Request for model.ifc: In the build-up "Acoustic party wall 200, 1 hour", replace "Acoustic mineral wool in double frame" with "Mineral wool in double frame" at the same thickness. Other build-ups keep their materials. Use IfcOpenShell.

First a look at what the model holds.

```python
import ifcopenshell
import ifcopenshell.util.element

model = ifcopenshell.open("model.ifc")
print(model.schema)
for layer_set in model.by_type("IfcMaterialLayerSet"):
    if layer_set.LayerSetName == "Acoustic party wall 200, 1 hour":
        for layer in layer_set.MaterialLayers:
            print(layer.id(), layer.Material and layer.Material.Name, layer.LayerThickness, sep=" | ")
        print(len(ifcopenshell.util.element.get_elements_by_material(model, layer_set)), "elements and types use it")
print(sorted(m.Name for m in model.by_type("IfcMaterial") if m.Name)[:60])
```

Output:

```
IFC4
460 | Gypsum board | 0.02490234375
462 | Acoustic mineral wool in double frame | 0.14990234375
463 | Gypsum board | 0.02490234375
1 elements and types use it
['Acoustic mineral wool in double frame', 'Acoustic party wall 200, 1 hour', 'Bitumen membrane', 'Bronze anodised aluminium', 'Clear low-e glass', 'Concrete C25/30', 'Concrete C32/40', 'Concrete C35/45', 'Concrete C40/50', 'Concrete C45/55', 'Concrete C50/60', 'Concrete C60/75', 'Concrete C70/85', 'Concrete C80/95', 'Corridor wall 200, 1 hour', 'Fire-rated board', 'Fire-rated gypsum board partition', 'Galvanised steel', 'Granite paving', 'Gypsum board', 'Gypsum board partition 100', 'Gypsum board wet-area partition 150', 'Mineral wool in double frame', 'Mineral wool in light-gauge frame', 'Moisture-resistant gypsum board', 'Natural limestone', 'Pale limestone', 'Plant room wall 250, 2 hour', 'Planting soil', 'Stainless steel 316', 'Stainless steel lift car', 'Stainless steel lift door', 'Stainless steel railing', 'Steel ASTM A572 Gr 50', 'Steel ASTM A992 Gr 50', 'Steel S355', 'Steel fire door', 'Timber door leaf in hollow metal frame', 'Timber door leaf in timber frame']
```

```python
import ifcopenshell
import ifcopenshell.api.material

model = ifcopenshell.open("model.ifc")

layer_set = next(s for s in model.by_type("IfcMaterialLayerSet") if s.LayerSetName == "Acoustic party wall 200, 1 hour")
layer = next(l for l in layer_set.MaterialLayers if l.Material and l.Material.Name == "Acoustic mineral wool in double frame")
material = next(m for m in model.by_type("IfcMaterial") if m.Name == "Mineral wool in double frame")

# Point this one layer at the other material; renaming the old one would change it everywhere.
ifcopenshell.api.material.edit_layer(model, layer=layer, attributes={}, material=material)

print([l.Material.Name if l.Material else None for l in layer_set.MaterialLayers])

model.write("model_v2.ifc")
```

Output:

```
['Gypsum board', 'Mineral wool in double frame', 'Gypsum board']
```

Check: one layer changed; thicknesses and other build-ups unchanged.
